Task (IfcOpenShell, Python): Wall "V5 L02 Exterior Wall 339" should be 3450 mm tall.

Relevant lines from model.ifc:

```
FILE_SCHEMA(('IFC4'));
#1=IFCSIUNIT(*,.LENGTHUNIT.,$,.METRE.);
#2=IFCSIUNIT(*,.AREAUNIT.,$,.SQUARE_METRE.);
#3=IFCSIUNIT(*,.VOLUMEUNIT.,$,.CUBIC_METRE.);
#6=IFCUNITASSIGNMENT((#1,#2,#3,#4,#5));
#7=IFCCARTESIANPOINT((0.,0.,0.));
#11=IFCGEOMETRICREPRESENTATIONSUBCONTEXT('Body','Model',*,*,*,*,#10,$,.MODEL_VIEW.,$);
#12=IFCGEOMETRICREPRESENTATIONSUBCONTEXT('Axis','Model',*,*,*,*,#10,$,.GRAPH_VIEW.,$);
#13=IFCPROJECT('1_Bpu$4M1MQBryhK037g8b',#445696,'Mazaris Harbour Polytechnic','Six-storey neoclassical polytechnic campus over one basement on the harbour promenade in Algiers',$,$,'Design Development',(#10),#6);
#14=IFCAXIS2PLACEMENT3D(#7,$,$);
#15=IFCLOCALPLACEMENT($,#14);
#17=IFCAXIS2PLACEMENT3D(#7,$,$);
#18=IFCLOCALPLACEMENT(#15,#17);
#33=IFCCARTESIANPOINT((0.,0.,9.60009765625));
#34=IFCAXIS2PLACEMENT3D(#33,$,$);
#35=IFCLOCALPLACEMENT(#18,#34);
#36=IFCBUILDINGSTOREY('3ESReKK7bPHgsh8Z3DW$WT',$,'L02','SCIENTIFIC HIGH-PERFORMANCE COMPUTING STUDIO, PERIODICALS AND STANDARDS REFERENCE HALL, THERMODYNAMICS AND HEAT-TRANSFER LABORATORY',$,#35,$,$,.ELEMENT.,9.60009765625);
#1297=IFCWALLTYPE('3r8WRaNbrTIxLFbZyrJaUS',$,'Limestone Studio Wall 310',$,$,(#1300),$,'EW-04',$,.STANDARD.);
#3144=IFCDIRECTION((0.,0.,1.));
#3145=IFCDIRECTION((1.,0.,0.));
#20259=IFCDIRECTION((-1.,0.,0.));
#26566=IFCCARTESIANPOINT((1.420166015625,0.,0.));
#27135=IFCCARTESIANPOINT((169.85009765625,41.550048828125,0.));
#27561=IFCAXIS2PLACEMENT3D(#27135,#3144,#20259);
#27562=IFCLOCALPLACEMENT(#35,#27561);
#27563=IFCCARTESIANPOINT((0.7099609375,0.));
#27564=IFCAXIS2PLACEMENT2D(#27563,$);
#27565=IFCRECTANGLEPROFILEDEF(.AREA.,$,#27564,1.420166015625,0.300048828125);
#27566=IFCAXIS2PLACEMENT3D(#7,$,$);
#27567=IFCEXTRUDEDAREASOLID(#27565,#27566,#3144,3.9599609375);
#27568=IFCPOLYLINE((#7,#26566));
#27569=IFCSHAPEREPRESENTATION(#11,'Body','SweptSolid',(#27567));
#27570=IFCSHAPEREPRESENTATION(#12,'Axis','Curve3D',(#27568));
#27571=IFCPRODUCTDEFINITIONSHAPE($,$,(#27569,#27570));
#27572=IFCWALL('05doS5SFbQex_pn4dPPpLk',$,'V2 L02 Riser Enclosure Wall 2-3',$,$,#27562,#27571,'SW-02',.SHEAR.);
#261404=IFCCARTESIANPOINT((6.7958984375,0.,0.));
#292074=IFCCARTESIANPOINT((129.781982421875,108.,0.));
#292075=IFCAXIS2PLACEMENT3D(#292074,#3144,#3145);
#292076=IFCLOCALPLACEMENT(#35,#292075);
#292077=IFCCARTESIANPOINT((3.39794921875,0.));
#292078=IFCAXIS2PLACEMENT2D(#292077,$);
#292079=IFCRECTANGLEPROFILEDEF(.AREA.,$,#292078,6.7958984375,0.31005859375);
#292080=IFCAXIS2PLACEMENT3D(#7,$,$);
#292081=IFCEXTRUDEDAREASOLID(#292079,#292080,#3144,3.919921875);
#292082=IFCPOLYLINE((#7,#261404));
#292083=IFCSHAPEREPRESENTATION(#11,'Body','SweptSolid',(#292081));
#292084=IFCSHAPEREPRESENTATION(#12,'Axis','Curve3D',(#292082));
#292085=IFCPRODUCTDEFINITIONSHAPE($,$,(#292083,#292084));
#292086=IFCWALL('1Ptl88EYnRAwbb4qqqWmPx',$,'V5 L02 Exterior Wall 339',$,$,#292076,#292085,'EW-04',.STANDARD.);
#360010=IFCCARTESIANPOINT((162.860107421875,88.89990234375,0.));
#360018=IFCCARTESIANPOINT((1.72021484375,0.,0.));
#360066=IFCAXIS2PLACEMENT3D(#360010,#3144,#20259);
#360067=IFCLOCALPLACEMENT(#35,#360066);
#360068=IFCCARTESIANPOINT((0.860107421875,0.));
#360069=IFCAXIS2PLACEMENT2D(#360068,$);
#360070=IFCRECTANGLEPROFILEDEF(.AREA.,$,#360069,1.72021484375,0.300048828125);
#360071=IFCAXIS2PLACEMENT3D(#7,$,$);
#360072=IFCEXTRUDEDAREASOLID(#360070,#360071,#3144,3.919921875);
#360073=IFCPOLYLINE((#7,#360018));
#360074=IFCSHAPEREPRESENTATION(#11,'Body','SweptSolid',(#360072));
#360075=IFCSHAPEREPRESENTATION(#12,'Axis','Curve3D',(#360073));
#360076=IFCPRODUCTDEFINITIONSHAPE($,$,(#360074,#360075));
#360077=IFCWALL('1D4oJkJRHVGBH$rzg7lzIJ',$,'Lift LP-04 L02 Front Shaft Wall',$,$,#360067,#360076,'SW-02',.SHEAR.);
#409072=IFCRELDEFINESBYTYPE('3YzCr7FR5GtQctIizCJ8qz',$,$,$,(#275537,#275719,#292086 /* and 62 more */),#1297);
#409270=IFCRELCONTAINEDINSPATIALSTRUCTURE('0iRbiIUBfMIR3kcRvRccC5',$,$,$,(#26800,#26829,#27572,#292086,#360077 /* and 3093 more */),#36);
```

```python
import ifcopenshell
import ifcopenshell.geom
import ifcopenshell.util.representation
import ifcopenshell.util.shape
import ifcopenshell.util.unit

model = ifcopenshell.open("model.ifc")
unit_scale = ifcopenshell.util.unit.calculate_unit_scale(model)
settings = ifcopenshell.geom.settings()


def volume(element):
    """Net volume in cubic metres, openings subtracted."""
    shape = ifcopenshell.geom.create_shape(settings, element)
    return ifcopenshell.util.shape.get_volume(shape.geometry)


wall = model.by_guid("1Ptl88EYnRAwbb4qqqWmPx")
before = volume(wall)

body = ifcopenshell.util.representation.get_representation(wall, "Model", "Body")
solid = body.Items[0]
old_height = solid.Depth
solid.Depth = 3.45 / unit_scale
after = volume(wall)

print(f"height {old_height:g} -> {solid.Depth:g}, volume {before:.3f} -> {after:.3f} m3")

model.write("model-out.ifc")
```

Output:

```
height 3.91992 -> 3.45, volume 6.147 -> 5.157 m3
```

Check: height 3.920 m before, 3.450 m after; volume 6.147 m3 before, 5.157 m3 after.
